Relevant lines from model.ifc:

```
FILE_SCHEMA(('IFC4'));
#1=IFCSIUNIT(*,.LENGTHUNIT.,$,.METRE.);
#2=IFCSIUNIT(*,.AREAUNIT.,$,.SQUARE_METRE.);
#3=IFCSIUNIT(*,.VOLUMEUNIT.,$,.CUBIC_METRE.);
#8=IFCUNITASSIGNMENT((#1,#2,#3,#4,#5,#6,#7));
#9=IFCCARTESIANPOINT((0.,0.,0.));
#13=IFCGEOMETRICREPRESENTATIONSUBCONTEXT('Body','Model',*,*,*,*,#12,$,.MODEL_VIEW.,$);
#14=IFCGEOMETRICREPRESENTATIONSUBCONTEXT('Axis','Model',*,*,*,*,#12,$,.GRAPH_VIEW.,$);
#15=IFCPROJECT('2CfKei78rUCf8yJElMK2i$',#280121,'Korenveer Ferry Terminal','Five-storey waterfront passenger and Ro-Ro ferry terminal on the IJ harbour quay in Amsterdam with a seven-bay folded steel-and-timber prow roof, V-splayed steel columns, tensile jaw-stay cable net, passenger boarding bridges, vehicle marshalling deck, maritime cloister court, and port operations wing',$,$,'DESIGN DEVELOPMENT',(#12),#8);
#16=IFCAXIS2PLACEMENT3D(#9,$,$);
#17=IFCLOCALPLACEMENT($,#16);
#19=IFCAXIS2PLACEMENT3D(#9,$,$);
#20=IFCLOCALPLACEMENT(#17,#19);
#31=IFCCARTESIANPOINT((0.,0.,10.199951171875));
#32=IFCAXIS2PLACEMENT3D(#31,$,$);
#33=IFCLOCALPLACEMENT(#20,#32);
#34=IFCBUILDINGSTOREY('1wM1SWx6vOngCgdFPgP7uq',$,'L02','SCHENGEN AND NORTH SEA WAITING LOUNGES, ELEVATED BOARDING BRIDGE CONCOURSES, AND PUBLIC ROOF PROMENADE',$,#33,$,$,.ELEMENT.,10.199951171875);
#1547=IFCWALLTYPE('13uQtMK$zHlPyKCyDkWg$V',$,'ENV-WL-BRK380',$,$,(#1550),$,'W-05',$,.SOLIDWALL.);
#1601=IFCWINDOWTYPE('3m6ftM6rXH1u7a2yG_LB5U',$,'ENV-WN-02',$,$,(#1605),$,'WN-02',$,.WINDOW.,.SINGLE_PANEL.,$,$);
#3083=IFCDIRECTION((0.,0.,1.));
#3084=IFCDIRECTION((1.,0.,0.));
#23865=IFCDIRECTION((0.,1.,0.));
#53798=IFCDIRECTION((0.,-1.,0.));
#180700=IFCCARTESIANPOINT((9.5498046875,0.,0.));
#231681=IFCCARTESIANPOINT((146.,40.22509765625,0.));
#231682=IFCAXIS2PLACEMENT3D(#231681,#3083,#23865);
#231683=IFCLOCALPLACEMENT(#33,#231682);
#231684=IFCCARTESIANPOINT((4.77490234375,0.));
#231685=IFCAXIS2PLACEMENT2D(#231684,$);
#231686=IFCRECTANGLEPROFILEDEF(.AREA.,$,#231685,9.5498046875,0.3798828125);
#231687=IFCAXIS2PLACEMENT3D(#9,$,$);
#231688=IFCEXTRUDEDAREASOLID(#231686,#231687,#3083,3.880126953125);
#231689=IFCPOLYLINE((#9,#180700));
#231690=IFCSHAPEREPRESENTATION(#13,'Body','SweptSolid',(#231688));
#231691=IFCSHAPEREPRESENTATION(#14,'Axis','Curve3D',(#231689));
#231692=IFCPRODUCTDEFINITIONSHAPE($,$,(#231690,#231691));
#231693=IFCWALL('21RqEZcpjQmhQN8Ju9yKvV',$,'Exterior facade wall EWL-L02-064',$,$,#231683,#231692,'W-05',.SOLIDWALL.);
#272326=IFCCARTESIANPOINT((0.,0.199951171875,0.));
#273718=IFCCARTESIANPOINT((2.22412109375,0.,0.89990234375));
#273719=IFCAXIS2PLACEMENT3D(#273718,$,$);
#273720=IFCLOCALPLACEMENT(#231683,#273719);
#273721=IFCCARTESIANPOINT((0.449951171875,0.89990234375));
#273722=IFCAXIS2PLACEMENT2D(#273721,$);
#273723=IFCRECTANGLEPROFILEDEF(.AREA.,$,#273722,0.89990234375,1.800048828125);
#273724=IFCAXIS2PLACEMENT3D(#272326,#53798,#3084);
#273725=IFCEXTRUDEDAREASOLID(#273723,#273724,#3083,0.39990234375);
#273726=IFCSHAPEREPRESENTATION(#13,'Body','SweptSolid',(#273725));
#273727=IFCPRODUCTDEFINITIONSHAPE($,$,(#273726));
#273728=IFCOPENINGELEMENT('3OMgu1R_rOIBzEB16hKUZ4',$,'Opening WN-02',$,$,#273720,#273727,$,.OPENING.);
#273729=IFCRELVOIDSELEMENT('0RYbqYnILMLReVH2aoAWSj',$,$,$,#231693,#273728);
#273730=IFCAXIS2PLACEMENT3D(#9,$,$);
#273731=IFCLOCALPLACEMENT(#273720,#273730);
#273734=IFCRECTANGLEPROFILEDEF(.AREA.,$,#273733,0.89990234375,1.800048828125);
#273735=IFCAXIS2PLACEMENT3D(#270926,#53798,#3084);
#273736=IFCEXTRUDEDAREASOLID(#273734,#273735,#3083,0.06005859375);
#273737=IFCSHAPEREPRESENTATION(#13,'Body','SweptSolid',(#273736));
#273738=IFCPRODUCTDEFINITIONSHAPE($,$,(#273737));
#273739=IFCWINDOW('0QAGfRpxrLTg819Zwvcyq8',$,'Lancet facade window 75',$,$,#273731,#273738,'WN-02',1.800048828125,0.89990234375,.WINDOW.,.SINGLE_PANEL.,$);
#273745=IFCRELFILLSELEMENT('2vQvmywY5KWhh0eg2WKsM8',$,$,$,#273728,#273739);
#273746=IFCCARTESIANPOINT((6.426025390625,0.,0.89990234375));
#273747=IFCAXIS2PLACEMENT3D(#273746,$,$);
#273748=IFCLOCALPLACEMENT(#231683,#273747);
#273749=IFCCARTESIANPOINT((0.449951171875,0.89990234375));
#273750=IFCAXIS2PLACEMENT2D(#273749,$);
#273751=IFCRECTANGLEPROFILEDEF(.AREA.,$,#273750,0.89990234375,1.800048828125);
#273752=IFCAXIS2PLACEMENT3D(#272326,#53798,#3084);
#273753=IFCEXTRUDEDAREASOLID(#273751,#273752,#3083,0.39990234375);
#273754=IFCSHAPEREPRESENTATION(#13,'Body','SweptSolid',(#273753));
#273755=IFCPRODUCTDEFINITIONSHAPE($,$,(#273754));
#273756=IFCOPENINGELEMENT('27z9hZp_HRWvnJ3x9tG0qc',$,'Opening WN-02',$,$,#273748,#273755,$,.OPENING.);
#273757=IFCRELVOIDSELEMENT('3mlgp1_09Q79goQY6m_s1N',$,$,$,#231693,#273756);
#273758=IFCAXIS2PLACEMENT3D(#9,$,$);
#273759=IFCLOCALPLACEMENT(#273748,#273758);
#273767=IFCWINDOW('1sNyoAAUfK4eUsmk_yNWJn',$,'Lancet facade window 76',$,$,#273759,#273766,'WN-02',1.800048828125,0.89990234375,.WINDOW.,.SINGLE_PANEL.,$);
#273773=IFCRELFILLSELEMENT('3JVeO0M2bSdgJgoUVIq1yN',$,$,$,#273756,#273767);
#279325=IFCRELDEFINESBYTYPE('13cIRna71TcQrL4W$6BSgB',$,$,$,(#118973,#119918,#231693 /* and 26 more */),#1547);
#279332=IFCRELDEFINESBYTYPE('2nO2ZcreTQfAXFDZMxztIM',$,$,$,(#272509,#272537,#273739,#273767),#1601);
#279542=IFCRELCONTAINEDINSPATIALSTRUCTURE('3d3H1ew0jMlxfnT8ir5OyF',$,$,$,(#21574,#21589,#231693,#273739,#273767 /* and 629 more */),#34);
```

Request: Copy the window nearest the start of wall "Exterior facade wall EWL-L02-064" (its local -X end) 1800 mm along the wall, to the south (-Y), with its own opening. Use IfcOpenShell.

```python
import ifcopenshell
import ifcopenshell.api.feature
import ifcopenshell.api.geometry
import ifcopenshell.api.root
import ifcopenshell.geom
import ifcopenshell.util.element
import ifcopenshell.util.placement
import ifcopenshell.util.shape
import ifcopenshell.util.unit

model = ifcopenshell.open("model.ifc")
unit_scale = ifcopenshell.util.unit.calculate_unit_scale(model)
settings = ifcopenshell.geom.settings()


def volume(element):
    """Net volume in cubic metres, openings subtracted."""
    shape = ifcopenshell.geom.create_shape(settings, element)
    return ifcopenshell.util.shape.get_volume(shape.geometry)


window = model.by_guid("0QAGfRpxrLTg819Zwvcyq8")
opening = window.FillsVoids[0].RelatingOpeningElement
wall = opening.VoidsElements[0].RelatingBuildingElement
before = volume(wall)
shift = ifcopenshell.util.placement.get_local_placement(wall.ObjectPlacement)[:3, 0] * -1.8 / unit_scale

# copy_class copies the void relationship, type, container and properties, but no geometry.
new_opening = ifcopenshell.api.root.copy_class(model, product=opening)
new_opening.Representation = ifcopenshell.util.element.copy_deep(
    model, opening.Representation, exclude=["IfcGeometricRepresentationContext", "IfcRepresentationMap"]
)
new_window = ifcopenshell.api.root.copy_class(model, product=window)
new_window.Representation = ifcopenshell.util.element.copy_deep(
    model, window.Representation, exclude=["IfcGeometricRepresentationContext", "IfcRepresentationMap"]
)
new_window.Tag = None
ifcopenshell.api.feature.add_filling(model, opening=new_opening, element=new_window)

for old, new in ((opening, new_opening), (window, new_window)):
    matrix = ifcopenshell.util.placement.get_local_placement(old.ObjectPlacement)
    matrix[:3, 3] += shift
    ifcopenshell.api.geometry.edit_object_placement(model, product=new, matrix=matrix, is_si=False)

after = volume(wall)

print(f"wall volume {before:.3f} -> {after:.3f} m3")

model.write("model_v2.ifc")
```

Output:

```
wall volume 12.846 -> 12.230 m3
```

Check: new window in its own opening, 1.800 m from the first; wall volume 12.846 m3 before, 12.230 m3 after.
